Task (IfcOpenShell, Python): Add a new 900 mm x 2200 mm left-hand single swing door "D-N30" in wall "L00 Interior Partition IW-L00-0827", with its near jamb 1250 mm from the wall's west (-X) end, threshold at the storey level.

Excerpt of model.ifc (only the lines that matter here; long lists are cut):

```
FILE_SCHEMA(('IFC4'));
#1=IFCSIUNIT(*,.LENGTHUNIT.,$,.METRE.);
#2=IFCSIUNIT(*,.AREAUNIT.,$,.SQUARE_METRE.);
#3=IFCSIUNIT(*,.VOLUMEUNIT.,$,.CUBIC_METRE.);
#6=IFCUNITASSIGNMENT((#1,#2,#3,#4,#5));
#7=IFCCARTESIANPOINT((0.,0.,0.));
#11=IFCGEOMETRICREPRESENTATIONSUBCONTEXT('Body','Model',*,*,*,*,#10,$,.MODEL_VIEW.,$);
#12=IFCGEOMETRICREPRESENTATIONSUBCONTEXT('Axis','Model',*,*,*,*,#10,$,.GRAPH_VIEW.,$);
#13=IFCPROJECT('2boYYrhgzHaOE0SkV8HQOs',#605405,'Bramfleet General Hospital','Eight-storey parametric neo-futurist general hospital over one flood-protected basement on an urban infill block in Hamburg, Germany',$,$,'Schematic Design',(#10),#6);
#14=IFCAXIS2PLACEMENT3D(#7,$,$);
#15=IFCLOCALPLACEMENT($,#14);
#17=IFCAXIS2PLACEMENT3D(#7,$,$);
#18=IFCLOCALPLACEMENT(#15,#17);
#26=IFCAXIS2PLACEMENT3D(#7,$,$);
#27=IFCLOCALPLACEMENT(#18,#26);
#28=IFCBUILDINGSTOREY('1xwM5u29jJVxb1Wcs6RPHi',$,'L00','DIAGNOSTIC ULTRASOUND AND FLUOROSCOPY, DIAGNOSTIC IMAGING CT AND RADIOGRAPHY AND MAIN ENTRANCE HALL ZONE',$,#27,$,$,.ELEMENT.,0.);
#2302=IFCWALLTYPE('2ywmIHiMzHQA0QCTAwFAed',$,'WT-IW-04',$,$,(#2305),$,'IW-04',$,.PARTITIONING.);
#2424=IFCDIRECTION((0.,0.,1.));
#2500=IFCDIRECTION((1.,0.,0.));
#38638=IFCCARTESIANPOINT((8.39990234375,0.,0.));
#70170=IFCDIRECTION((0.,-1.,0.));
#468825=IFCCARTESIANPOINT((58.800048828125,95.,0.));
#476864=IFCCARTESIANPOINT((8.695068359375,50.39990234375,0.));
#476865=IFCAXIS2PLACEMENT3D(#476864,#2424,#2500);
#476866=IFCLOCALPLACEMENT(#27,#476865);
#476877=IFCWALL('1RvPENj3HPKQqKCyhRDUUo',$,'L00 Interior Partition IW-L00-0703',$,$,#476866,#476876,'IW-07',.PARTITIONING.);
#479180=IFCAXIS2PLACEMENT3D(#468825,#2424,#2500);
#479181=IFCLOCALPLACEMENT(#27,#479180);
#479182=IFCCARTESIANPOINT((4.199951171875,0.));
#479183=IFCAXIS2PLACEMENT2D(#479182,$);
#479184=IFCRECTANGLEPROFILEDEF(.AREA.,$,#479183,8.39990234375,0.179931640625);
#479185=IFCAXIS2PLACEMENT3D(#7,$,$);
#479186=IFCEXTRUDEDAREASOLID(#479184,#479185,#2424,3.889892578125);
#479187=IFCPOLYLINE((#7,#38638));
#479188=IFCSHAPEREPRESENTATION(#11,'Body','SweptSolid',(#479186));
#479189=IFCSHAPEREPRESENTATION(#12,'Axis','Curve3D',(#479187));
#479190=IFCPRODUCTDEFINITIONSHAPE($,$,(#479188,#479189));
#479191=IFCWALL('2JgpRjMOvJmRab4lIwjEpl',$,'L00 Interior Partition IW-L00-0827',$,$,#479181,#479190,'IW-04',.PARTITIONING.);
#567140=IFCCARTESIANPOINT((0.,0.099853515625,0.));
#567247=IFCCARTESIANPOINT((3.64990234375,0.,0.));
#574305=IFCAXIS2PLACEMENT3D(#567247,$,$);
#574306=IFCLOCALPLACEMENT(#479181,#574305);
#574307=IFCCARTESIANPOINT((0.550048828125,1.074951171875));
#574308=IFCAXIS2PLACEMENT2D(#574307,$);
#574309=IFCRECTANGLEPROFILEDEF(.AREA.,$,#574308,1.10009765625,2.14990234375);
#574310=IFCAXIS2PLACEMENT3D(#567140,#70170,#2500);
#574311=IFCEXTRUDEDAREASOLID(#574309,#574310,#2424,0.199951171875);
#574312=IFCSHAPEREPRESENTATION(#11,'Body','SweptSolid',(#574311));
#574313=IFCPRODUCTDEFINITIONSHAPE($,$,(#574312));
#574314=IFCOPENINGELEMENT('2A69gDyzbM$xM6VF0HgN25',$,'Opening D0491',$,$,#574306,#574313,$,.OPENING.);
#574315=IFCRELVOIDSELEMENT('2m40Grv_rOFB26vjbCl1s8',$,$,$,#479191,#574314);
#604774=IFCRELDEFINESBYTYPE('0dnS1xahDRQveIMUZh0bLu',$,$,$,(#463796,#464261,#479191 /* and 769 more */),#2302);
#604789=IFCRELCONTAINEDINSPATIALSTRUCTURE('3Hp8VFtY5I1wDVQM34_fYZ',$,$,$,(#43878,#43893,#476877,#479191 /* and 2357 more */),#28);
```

```python
import numpy as np
import ifcopenshell
import ifcopenshell.api.feature
import ifcopenshell.api.geometry
import ifcopenshell.api.root
import ifcopenshell.api.spatial
import ifcopenshell.geom
import ifcopenshell.util.element
import ifcopenshell.util.placement
import ifcopenshell.util.representation
import ifcopenshell.util.shape
import ifcopenshell.util.unit

model = ifcopenshell.open("model.ifc")
unit_scale = ifcopenshell.util.unit.calculate_unit_scale(model)
settings = ifcopenshell.geom.settings()


def volume(element):
    """Net volume in cubic metres, openings subtracted."""
    shape = ifcopenshell.geom.create_shape(settings, element)
    return ifcopenshell.util.shape.get_volume(shape.geometry)


wall = model.by_id(479191)
storey = ifcopenshell.util.element.get_container(wall, ifc_class="IfcBuildingStorey")
context = ifcopenshell.util.representation.get_context(model, "Model", "Body", "MODEL_VIEW")
before = volume(wall)

width, height, from_end, sill = 0.9, 2.2, 1.25, 0.0  # metres

# The wall runs along its own X axis, and the end named is its -X end.
wall_shape = ifcopenshell.geom.create_shape(settings, wall)
x, y, z = ifcopenshell.util.shape.get_vertices(wall_shape.geometry).T
start = x.min() + from_end
face, thickness = float(y.min()), float(y.max() - y.min())
wall_matrix = ifcopenshell.util.placement.get_local_placement(wall.ObjectPlacement)
level = ifcopenshell.util.placement.get_local_placement(storey.ObjectPlacement)[2, 3]


def in_wall(x, y):
    """Placement at x, y metres in the wall's axes, at sill height."""
    matrix = wall_matrix.copy()
    matrix[:, 3] = wall_matrix @ np.array([x / unit_scale, y / unit_scale, 0.0, 1.0])
    matrix[2, 3] = level + sill / unit_scale
    return matrix


# Opening: a box that overshoots both wall faces by 50 mm.
opening = ifcopenshell.api.root.create_entity(model, ifc_class="IfcOpeningElement", predefined_type="OPENING")
box = ifcopenshell.api.geometry.add_wall_representation(
    model, context=context, length=width, height=height, thickness=thickness + 0.1
)
ifcopenshell.api.geometry.assign_representation(model, product=opening, representation=box)
ifcopenshell.api.geometry.edit_object_placement(model, product=opening, matrix=in_wall(start, face - 0.05), is_si=False)
ifcopenshell.api.feature.add_feature(model, feature=opening, element=wall)

door = ifcopenshell.api.root.create_entity(model, ifc_class="IfcDoor", name="D-N30", predefined_type="DOOR")
door.OverallWidth, door.OverallHeight = width / unit_scale, height / unit_scale
door.OperationType = "SINGLE_SWING_LEFT"
body = ifcopenshell.api.geometry.add_door_representation(
    model,
    context=context,
    overall_width=door.OverallWidth,
    overall_height=door.OverallHeight,
    operation_type="SINGLE_SWING_LEFT",
    lining_properties={"LiningDepth": thickness / unit_scale, "ThresholdDepth": thickness / unit_scale},
)
ifcopenshell.api.geometry.assign_representation(model, product=door, representation=body)
ifcopenshell.api.spatial.assign_container(model, products=[door], relating_structure=storey)
ifcopenshell.api.feature.add_filling(model, opening=opening, element=door)

# The lining spans the wall, so the door starts at the wall face.
ifcopenshell.api.geometry.edit_object_placement(model, product=door, matrix=in_wall(start, face), is_si=False)

after = volume(wall)

print(f"wall volume {before:.3f} -> {after:.3f} m3")

model.write("model_updated.ifc")
```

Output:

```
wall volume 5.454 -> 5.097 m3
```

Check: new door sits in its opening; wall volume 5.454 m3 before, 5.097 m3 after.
